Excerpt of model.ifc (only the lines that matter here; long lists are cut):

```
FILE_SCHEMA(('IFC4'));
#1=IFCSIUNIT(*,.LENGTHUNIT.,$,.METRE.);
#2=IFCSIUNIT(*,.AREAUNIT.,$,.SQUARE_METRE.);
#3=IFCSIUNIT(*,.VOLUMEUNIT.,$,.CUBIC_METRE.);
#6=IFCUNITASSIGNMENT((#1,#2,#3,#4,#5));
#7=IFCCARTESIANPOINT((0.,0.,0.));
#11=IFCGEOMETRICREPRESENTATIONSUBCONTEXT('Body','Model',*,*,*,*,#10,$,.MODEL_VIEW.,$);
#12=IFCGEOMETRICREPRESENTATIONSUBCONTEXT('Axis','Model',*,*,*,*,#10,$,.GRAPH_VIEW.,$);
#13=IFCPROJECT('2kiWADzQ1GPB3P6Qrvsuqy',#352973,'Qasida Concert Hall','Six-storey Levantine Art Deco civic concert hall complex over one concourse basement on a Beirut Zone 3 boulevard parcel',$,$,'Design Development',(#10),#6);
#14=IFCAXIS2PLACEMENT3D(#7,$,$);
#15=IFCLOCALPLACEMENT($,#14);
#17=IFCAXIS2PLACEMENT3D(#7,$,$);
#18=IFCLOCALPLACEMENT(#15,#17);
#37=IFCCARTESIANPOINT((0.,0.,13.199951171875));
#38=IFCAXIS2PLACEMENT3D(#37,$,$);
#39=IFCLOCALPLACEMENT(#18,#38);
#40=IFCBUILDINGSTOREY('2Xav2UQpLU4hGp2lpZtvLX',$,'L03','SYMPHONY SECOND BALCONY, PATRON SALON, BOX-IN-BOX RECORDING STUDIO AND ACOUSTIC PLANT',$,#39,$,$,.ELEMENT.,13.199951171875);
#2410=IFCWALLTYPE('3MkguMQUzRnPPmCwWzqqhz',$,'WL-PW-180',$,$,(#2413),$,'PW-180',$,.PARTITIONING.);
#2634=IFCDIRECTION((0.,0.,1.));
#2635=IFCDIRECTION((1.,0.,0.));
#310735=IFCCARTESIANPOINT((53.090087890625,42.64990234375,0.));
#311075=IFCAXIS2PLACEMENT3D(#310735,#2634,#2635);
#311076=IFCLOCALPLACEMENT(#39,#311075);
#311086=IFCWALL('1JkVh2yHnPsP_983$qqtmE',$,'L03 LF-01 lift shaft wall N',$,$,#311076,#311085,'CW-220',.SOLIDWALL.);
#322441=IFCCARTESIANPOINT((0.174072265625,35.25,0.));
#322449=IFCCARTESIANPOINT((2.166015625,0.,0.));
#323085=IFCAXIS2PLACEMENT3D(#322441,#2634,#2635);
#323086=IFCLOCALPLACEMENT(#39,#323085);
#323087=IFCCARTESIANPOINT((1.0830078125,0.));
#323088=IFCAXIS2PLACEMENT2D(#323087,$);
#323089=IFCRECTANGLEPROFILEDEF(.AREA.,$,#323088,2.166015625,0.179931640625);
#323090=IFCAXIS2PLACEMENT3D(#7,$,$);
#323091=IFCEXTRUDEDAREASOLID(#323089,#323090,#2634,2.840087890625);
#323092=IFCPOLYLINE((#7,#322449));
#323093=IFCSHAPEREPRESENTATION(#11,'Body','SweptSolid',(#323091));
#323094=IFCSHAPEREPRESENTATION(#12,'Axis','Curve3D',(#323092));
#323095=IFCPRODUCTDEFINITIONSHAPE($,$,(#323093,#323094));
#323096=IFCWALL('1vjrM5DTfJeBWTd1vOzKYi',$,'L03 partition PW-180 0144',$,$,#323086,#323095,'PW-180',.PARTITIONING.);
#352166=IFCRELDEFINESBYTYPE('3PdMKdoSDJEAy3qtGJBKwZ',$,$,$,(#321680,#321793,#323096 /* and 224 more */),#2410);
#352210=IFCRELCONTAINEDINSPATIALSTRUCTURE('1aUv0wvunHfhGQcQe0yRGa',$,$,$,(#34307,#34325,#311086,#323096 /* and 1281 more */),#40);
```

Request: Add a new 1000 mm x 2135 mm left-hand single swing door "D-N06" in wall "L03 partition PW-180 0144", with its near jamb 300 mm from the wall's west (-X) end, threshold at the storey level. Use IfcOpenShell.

```python
import numpy as np
import ifcopenshell
import ifcopenshell.api.feature
import ifcopenshell.api.geometry
import ifcopenshell.api.root
import ifcopenshell.api.spatial
import ifcopenshell.geom
import ifcopenshell.util.element
import ifcopenshell.util.placement
import ifcopenshell.util.representation
import ifcopenshell.util.shape
import ifcopenshell.util.unit

model = ifcopenshell.open("model.ifc")
unit_scale = ifcopenshell.util.unit.calculate_unit_scale(model)
settings = ifcopenshell.geom.settings()


def volume(element):
    """Net volume in cubic metres, openings subtracted."""
    shape = ifcopenshell.geom.create_shape(settings, element)
    return ifcopenshell.util.shape.get_volume(shape.geometry)


wall = model.by_guid("1vjrM5DTfJeBWTd1vOzKYi")
storey = ifcopenshell.util.element.get_container(wall, ifc_class="IfcBuildingStorey")
context = ifcopenshell.util.representation.get_context(model, "Model", "Body", "MODEL_VIEW")
before = volume(wall)

width, height, from_end, sill = 1, 2.135, 0.3, 0.0  # metres

# The wall runs along its own X axis, and the end named is its -X end.
wall_shape = ifcopenshell.geom.create_shape(settings, wall)
x, y, z = ifcopenshell.util.shape.get_vertices(wall_shape.geometry).T
start = x.min() + from_end
face, thickness = float(y.min()), float(y.max() - y.min())
wall_matrix = ifcopenshell.util.placement.get_local_placement(wall.ObjectPlacement)
level = ifcopenshell.util.placement.get_local_placement(storey.ObjectPlacement)[2, 3]


def in_wall(x, y):
    """Placement at x, y metres in the wall's axes, at sill height."""
    matrix = wall_matrix.copy()
    matrix[:, 3] = wall_matrix @ np.array([x / unit_scale, y / unit_scale, 0.0, 1.0])
    matrix[2, 3] = level + sill / unit_scale
    return matrix


# Opening: a box that overshoots both wall faces by 50 mm.
opening = ifcopenshell.api.root.create_entity(model, ifc_class="IfcOpeningElement", predefined_type="OPENING")
box = ifcopenshell.api.geometry.add_wall_representation(
    model, context=context, length=width, height=height, thickness=thickness + 0.1
)
ifcopenshell.api.geometry.assign_representation(model, product=opening, representation=box)
ifcopenshell.api.geometry.edit_object_placement(model, product=opening, matrix=in_wall(start, face - 0.05), is_si=False)
ifcopenshell.api.feature.add_feature(model, feature=opening, element=wall)

door = ifcopenshell.api.root.create_entity(model, ifc_class="IfcDoor", name="D-N06", predefined_type="DOOR")
door.OverallWidth, door.OverallHeight = width / unit_scale, height / unit_scale
door.OperationType = "SINGLE_SWING_LEFT"
body = ifcopenshell.api.geometry.add_door_representation(
    model,
    context=context,
    overall_width=door.OverallWidth,
    overall_height=door.OverallHeight,
    operation_type="SINGLE_SWING_LEFT",
    lining_properties={"LiningDepth": thickness / unit_scale, "ThresholdDepth": thickness / unit_scale},
)
ifcopenshell.api.geometry.assign_representation(model, product=door, representation=body)
ifcopenshell.api.spatial.assign_container(model, products=[door], relating_structure=storey)
ifcopenshell.api.feature.add_filling(model, opening=opening, element=door)

# The lining spans the wall, so the door starts at the wall face.
ifcopenshell.api.geometry.edit_object_placement(model, product=door, matrix=in_wall(start, face), is_si=False)

after = volume(wall)

print(f"wall volume {before:.3f} -> {after:.3f} m3")

model.write("model_v2.ifc")
```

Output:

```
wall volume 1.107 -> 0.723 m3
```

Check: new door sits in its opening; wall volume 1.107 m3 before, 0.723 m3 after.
